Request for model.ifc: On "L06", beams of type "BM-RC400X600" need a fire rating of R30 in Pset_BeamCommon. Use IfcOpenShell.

First a look at what the model holds.

```python
import ifcopenshell
import ifcopenshell.util.element

model = ifcopenshell.open("model.ifc")
print(model.schema)
storey = next(s for s in model.by_type("IfcBuildingStorey") if s.Name == "L06")
beams = [e for e in ifcopenshell.util.element.get_decomposition(storey) if e.is_a("IfcBeam")]
seen = {}
for e in beams:
    element_type = ifcopenshell.util.element.get_type(e)
    key = (element_type.Name if element_type != e and element_type else None, ifcopenshell.util.element.get_pset(e, "Pset_BeamCommon", "FireRating"))
    seen[key] = seen.get(key, 0) + 1
for (name, value), count in sorted(seen.items(), key=str):
    print(count, "x", name, "|", value)
```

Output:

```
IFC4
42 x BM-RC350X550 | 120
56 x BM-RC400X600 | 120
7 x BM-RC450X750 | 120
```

```python
import ifcopenshell
import ifcopenshell.api.pset
import ifcopenshell.util.element

model = ifcopenshell.open("model.ifc")

storey = next(s for s in model.by_type("IfcBuildingStorey") if s.Name == "L06")
beams = [e for e in ifcopenshell.util.element.get_decomposition(storey) if e.is_a("IfcBeam")]

count = 0
for e in beams:
    element_type = ifcopenshell.util.element.get_type(e)
    if element_type in (None, e) or element_type.Name != "BM-RC400X600":
        continue
    # add_pset returns the element's existing set when there is one.
    pset = ifcopenshell.api.pset.add_pset(model, product=e, name="Pset_BeamCommon")
    ifcopenshell.api.pset.edit_pset(model, pset=pset, properties={"FireRating": "R30"})
    count += 1

print(count, "beams updated")

model.write("model_rev.ifc")
```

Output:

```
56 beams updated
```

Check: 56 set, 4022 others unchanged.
